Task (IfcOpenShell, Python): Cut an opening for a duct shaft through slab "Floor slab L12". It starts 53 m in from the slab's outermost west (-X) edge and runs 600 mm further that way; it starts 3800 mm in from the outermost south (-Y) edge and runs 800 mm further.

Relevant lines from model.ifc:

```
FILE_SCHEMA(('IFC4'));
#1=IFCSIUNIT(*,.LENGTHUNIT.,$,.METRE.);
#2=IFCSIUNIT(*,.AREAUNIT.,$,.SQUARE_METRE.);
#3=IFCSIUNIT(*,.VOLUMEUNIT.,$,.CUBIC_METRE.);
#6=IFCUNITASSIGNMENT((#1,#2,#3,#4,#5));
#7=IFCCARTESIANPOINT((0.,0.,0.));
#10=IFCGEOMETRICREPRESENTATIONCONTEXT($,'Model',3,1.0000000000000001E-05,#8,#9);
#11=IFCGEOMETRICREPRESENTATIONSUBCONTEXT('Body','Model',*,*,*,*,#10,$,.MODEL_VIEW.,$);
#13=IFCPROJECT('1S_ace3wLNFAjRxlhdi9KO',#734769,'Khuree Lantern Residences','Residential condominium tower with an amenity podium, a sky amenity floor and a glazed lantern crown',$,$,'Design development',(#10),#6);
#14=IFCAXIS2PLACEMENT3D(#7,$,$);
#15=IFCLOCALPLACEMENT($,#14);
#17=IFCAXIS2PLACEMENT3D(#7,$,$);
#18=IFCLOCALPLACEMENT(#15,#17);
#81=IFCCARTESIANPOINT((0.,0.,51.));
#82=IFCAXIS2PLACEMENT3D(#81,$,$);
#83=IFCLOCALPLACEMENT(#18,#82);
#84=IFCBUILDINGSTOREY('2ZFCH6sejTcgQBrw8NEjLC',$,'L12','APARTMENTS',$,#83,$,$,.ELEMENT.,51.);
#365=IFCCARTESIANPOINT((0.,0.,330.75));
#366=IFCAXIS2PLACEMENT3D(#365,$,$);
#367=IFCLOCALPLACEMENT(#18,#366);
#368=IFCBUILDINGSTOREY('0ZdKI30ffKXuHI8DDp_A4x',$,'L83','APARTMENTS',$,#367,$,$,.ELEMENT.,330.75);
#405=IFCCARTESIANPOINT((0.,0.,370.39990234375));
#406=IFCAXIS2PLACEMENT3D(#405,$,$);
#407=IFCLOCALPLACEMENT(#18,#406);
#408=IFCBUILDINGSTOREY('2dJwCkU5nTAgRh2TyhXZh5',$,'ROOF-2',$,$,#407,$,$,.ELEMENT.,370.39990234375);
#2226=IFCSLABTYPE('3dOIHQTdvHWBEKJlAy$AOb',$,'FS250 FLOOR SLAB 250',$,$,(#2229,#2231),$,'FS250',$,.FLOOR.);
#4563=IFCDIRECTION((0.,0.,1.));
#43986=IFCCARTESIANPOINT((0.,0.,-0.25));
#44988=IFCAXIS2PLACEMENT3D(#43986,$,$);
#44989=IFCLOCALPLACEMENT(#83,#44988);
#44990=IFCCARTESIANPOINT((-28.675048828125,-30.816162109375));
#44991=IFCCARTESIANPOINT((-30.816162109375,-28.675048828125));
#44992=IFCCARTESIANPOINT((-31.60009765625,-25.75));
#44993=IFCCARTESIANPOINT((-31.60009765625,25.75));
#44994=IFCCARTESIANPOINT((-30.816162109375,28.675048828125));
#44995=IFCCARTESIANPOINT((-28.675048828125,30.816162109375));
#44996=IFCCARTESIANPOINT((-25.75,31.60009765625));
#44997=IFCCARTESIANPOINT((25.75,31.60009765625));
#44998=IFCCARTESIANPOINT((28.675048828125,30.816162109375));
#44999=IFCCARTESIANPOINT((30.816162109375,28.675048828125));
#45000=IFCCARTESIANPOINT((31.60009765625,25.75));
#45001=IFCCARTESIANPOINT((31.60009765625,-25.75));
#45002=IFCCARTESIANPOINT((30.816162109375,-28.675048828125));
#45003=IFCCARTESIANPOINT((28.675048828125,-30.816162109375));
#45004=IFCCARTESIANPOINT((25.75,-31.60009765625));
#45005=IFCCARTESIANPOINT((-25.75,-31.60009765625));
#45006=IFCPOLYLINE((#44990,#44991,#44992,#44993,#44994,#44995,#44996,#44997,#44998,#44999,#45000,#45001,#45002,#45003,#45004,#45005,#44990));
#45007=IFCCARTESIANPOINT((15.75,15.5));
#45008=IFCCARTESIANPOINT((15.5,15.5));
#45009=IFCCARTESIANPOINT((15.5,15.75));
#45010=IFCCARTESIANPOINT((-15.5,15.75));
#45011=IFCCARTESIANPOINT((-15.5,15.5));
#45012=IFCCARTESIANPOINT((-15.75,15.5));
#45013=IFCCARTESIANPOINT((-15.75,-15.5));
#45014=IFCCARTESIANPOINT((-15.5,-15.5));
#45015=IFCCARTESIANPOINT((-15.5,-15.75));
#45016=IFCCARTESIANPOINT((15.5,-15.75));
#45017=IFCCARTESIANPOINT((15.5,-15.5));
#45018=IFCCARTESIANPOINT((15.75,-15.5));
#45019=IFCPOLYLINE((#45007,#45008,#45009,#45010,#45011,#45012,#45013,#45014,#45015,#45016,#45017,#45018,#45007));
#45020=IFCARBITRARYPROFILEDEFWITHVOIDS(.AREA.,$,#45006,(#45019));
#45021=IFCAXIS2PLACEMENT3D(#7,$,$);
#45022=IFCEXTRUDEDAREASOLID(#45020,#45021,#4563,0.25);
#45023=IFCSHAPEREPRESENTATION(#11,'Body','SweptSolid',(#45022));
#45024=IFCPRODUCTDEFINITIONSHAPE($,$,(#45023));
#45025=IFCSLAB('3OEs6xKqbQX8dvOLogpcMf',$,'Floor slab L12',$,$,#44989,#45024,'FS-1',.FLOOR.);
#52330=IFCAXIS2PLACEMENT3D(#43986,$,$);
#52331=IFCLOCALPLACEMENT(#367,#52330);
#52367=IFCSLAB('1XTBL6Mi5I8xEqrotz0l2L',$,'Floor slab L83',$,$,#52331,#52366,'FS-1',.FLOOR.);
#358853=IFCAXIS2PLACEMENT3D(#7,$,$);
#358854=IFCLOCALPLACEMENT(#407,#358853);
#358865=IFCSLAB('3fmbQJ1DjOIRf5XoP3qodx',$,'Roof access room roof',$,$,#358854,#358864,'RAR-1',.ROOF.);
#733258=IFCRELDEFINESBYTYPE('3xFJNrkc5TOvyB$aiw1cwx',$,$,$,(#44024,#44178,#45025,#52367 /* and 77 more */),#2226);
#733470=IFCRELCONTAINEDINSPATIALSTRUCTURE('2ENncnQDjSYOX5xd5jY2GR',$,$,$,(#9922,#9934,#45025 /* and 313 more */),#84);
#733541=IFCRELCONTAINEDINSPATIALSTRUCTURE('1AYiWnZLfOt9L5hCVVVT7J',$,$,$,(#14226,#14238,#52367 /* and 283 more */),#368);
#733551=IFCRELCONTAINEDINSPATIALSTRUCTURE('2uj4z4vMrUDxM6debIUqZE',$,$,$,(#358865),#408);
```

```python
import numpy as np
import ifcopenshell
import ifcopenshell.api.feature
import ifcopenshell.api.geometry
import ifcopenshell.api.root
import ifcopenshell.geom
import ifcopenshell.util.placement
import ifcopenshell.util.representation
import ifcopenshell.util.shape
import ifcopenshell.util.unit

model = ifcopenshell.open("model.ifc")
unit_scale = ifcopenshell.util.unit.calculate_unit_scale(model)
settings = ifcopenshell.geom.settings()


def volume(element):
    """Net volume in cubic metres, openings subtracted."""
    shape = ifcopenshell.geom.create_shape(settings, element)
    return ifcopenshell.util.shape.get_volume(shape.geometry)


slab = model.by_id(45025)
before = volume(slab)

# Extent in the slab's own axes, in metres. The edges named are its -X and -Y sides.
slab_shape = ifcopenshell.geom.create_shape(settings, slab)
vertices = ifcopenshell.util.shape.get_vertices(slab_shape.geometry)
x_min, y_min, bottom = vertices.min(axis=0)
top = vertices[:, 2].max()

opening = ifcopenshell.api.root.create_entity(model, ifc_class="IfcOpeningElement", name="Duct shaft opening", predefined_type="OPENING")
context = ifcopenshell.util.representation.get_context(model, "Model", "Body", "MODEL_VIEW")
width, depth = 0.6, 0.8
outline = [(0.0, 0.0), (width, 0.0), (width, depth), (0.0, depth), (0.0, 0.0)]
# Overshoot both faces by 50 mm so the cut is clean.
shape = ifcopenshell.api.geometry.add_slab_representation(
    model, context=context, depth=top - bottom + 0.1, polyline=outline
)
ifcopenshell.api.geometry.assign_representation(model, product=opening, representation=shape)

matrix = ifcopenshell.util.placement.get_local_placement(slab.ObjectPlacement)
matrix[:, 3] = matrix @ np.append(np.array([x_min + 53, y_min + 3.8, bottom - 0.05]) / unit_scale, 1.0)
ifcopenshell.api.geometry.edit_object_placement(model, product=opening, matrix=matrix, is_si=False)
ifcopenshell.api.feature.add_feature(model, feature=opening, element=slab)

after = volume(slab)

print(f"slab volume {before:.3f} -> {after:.3f} m3")

model.write("model_rev.ifc")
```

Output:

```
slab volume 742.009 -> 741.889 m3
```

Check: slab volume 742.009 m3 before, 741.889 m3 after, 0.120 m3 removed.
